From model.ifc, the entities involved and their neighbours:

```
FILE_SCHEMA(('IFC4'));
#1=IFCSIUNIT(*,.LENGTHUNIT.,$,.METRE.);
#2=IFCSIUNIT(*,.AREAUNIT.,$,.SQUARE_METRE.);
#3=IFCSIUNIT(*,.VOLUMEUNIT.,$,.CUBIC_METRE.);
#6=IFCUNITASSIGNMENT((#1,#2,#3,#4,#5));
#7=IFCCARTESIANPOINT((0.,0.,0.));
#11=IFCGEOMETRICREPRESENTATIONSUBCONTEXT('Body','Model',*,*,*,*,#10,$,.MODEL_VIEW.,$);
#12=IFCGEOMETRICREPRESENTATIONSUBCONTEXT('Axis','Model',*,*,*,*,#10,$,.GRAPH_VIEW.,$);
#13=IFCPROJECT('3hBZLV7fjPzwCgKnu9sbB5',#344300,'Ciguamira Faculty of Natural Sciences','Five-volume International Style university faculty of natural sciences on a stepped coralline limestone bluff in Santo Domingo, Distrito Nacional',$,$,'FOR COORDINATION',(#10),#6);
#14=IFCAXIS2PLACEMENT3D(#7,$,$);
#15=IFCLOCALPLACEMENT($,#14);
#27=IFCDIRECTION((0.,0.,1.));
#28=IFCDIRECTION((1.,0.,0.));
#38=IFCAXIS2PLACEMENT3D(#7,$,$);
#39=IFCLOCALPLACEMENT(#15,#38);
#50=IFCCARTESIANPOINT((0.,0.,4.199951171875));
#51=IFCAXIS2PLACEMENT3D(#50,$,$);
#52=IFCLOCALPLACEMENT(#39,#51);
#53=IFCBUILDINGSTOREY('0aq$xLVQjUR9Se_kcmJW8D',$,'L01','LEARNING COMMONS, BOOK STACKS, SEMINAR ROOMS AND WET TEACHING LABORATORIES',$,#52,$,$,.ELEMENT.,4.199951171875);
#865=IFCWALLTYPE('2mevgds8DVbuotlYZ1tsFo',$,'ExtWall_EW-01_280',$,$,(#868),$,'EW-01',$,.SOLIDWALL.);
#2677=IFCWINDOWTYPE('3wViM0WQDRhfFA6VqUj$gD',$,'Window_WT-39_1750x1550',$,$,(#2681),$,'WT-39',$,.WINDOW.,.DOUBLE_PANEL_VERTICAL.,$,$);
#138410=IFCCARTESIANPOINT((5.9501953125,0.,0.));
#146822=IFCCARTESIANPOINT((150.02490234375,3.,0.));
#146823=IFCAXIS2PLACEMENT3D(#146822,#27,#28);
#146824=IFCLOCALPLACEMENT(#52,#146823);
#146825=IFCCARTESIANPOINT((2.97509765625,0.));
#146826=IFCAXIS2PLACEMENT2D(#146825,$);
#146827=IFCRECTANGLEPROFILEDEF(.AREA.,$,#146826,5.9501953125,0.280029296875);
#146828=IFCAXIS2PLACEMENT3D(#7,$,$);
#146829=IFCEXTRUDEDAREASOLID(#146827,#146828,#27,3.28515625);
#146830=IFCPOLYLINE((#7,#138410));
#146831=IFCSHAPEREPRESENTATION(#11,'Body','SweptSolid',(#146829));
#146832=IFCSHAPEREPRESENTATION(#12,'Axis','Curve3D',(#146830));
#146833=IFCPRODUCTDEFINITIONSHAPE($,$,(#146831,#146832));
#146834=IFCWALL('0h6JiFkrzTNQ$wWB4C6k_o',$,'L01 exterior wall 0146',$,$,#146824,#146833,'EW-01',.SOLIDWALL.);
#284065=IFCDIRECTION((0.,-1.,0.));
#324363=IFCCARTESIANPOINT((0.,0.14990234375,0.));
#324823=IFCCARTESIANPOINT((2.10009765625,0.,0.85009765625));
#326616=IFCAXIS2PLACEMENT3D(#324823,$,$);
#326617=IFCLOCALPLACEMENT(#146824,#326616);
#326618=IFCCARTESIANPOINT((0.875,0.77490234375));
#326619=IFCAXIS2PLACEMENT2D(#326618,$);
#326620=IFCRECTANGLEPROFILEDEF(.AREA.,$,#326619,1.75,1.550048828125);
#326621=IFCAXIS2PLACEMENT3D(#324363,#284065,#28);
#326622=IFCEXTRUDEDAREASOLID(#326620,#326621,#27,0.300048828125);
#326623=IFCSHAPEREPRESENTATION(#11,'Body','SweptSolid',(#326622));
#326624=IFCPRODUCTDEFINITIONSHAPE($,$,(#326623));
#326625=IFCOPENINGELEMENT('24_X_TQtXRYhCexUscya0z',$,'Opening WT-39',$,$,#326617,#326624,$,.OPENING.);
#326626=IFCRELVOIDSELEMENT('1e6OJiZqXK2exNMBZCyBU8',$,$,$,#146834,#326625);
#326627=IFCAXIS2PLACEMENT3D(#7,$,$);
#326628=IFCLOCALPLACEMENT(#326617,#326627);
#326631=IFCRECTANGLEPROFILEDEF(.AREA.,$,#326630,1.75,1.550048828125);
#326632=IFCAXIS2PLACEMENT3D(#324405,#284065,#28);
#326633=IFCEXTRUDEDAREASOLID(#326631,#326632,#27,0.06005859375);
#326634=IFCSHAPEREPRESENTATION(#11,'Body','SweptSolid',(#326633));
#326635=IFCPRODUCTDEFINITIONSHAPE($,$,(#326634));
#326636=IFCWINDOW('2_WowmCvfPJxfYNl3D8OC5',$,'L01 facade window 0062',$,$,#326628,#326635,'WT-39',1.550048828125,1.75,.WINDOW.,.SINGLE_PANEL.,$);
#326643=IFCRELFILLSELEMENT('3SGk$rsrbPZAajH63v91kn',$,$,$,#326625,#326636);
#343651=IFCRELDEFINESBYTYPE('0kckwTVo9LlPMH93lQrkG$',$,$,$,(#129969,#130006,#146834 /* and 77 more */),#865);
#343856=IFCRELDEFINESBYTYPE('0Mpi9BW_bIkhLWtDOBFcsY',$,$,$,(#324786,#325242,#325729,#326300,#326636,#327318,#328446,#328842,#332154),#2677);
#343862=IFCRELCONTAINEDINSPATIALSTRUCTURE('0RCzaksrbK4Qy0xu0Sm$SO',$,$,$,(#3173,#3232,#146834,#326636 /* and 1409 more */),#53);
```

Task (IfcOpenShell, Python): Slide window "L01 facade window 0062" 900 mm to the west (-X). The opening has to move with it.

```python
import ifcopenshell
import ifcopenshell.api.geometry
import ifcopenshell.util.placement

model = ifcopenshell.open("model.ifc")

window = model.by_guid("2_WowmCvfPJxfYNl3D8OC5")
opening = window.FillsVoids[0].RelatingOpeningElement
wall = opening.VoidsElements[0].RelatingBuildingElement

wall_matrix = ifcopenshell.util.placement.get_local_placement(wall.ObjectPlacement)
shift = wall_matrix[:3, 0] * -0.9
before = ifcopenshell.util.placement.get_local_placement(window.ObjectPlacement)[:3, 3].copy()

# The window is placed relative to its opening, so it follows when the opening moves.
matrix = ifcopenshell.util.placement.get_local_placement(opening.ObjectPlacement)
matrix[:3, 3] += shift
ifcopenshell.api.geometry.edit_object_placement(
    model, product=opening, matrix=matrix, is_si=False, should_transform_children=True
)

after = ifcopenshell.util.placement.get_local_placement(window.ObjectPlacement)[:3, 3]
print("window moved by", (after - before).round(3) + 0.0)

model.write("model_v2.ifc")
```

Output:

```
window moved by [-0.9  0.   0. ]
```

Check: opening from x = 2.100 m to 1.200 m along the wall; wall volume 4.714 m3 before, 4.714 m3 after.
